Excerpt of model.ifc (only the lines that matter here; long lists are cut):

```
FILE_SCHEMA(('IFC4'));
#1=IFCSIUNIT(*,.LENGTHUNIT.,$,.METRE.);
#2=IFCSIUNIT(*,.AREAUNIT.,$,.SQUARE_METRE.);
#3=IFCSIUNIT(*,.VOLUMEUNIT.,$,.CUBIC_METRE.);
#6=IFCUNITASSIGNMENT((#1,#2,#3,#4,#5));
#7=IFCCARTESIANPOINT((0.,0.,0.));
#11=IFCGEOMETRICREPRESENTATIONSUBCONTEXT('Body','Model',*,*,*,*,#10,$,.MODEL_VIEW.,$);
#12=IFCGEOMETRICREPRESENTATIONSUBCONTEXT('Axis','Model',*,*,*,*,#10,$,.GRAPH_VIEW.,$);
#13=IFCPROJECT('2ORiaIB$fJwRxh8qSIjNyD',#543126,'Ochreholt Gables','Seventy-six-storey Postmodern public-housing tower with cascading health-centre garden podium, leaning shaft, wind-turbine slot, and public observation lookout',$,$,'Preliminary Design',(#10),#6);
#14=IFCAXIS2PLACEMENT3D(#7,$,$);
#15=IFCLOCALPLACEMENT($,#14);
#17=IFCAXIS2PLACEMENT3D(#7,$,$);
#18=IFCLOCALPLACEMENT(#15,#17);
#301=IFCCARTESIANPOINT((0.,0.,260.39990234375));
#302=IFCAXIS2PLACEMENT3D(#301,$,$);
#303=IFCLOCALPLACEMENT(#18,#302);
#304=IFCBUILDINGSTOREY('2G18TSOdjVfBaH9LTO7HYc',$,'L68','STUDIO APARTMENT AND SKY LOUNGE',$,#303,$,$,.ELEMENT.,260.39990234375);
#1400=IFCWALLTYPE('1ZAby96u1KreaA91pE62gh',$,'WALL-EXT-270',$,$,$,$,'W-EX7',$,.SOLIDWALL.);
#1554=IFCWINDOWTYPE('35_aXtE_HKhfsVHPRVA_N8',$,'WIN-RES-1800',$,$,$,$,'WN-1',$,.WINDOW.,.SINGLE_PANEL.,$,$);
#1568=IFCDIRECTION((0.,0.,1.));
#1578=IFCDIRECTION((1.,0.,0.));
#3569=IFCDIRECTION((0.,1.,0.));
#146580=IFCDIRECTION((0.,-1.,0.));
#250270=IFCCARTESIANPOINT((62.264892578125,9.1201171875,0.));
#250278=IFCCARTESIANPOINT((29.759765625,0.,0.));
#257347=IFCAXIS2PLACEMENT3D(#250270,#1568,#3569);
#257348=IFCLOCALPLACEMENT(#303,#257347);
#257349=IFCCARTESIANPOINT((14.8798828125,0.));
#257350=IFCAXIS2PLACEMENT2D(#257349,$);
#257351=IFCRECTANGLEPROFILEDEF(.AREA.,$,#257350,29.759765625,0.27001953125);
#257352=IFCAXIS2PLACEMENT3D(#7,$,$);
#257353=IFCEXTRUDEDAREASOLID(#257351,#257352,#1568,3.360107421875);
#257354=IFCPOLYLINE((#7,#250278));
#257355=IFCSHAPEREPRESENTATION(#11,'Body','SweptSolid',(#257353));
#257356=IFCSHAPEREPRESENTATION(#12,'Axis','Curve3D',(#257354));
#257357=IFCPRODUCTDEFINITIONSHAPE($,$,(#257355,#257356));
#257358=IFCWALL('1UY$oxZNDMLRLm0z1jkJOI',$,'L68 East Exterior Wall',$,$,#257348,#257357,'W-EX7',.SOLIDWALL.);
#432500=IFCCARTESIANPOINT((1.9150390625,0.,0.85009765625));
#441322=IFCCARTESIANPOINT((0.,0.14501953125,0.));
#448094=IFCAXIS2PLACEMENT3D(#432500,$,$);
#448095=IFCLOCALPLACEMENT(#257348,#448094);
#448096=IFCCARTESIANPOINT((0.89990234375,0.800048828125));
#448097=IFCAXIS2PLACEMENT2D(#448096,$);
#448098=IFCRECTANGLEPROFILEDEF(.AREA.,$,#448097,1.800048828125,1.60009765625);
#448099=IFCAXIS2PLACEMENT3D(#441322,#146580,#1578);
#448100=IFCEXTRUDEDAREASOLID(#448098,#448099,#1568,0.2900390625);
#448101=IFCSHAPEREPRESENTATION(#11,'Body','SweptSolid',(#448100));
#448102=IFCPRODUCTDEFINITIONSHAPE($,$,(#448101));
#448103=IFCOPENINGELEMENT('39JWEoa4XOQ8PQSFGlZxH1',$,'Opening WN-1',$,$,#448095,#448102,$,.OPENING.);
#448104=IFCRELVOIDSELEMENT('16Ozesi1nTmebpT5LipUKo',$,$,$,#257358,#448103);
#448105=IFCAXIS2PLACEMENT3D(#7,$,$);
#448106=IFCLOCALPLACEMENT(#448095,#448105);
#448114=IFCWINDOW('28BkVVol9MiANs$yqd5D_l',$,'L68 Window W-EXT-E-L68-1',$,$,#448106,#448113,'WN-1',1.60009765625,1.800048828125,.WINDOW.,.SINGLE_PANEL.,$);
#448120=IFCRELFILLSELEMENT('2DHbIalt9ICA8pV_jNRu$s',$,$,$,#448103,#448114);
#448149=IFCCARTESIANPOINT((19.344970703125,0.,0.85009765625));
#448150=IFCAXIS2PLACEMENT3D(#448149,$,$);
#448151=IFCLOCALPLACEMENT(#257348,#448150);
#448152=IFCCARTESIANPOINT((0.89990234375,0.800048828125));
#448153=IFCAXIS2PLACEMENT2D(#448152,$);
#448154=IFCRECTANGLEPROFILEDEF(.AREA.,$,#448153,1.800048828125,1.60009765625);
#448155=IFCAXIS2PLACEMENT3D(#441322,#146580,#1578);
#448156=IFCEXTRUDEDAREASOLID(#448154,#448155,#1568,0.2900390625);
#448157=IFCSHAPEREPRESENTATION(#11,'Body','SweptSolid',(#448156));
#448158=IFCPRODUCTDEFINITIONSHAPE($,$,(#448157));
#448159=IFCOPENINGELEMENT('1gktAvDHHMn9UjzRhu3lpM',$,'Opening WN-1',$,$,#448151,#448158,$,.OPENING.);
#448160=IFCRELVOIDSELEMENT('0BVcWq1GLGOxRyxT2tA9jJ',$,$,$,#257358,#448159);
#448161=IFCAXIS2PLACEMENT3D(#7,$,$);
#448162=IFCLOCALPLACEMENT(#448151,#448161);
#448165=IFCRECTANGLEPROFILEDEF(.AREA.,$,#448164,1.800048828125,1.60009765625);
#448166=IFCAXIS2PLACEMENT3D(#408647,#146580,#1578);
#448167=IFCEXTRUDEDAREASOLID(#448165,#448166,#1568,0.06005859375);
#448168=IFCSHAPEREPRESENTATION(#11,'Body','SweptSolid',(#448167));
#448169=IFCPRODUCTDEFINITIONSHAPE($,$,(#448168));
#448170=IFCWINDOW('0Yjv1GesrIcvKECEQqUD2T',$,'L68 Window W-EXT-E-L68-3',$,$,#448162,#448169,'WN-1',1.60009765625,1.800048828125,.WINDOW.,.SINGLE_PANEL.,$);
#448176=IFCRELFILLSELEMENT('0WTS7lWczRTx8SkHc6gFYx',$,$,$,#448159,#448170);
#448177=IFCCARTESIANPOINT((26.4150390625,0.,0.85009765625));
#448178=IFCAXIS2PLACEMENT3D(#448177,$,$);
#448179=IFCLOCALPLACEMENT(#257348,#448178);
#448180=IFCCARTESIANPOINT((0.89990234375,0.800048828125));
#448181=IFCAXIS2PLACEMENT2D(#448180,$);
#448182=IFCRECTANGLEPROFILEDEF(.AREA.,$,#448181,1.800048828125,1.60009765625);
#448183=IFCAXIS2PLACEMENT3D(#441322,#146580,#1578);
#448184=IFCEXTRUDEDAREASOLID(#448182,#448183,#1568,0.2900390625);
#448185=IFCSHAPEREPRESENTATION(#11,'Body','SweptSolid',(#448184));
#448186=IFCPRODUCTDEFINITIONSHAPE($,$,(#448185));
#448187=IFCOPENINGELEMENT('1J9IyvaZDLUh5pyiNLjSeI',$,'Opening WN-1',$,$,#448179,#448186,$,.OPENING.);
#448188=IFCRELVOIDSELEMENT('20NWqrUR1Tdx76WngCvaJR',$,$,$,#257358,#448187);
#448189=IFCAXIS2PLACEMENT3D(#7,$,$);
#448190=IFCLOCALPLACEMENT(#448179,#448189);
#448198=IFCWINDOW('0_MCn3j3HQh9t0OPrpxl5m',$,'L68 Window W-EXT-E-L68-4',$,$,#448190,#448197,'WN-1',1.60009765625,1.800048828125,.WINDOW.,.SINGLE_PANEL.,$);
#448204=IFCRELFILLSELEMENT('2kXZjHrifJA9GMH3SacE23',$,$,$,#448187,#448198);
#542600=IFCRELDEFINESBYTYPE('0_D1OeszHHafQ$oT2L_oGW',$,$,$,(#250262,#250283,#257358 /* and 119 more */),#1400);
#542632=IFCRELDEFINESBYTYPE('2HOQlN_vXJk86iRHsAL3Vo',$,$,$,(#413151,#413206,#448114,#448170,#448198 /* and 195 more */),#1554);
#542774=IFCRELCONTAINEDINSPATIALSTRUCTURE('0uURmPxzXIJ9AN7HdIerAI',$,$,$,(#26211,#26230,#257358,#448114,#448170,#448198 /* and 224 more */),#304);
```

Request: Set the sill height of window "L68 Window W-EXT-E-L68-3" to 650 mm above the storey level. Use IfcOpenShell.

```python
import numpy as np
import ifcopenshell
import ifcopenshell.api.geometry
import ifcopenshell.geom
import ifcopenshell.util.element
import ifcopenshell.util.placement
import ifcopenshell.util.shape
import ifcopenshell.util.unit

model = ifcopenshell.open("model.ifc")
unit_scale = ifcopenshell.util.unit.calculate_unit_scale(model)

window = model.by_guid("0Yjv1GesrIcvKECEQqUD2T")
opening = window.FillsVoids[0].RelatingOpeningElement
storey = ifcopenshell.util.element.get_container(window, ifc_class="IfcBuildingStorey")
level = ifcopenshell.util.placement.get_local_placement(storey.ObjectPlacement)[2, 3]

# The opening's origin need not be at the sill, so measure its lowest point.
shape = ifcopenshell.geom.create_shape(ifcopenshell.geom.settings(), opening)
bottom = ifcopenshell.util.shape.get_shape_bottom_elevation(shape, shape.geometry) / unit_scale
dz = level + 0.65 - bottom

shift = np.array([0.0, 0.0, dz])
# The window is placed relative to its opening, so it follows when the opening moves.
matrix = ifcopenshell.util.placement.get_local_placement(opening.ObjectPlacement)
matrix[:3, 3] += shift
ifcopenshell.api.geometry.edit_object_placement(
    model, product=opening, matrix=matrix, is_si=False, should_transform_children=True
)

print(f"moved by {dz * unit_scale:+.3f} m")

model.write("model_v2.ifc")
```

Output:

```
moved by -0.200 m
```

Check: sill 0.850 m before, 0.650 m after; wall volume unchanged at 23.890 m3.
